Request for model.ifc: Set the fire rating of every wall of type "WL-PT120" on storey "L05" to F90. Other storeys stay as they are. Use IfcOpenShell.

First a look at what the model holds.

```python
import ifcopenshell
import ifcopenshell.util.element

model = ifcopenshell.open("model.ifc")
print(model.schema)
storey = next(s for s in model.by_type("IfcBuildingStorey") if s.Name == "L05")
walls = [e for e in ifcopenshell.util.element.get_decomposition(storey) if e.is_a("IfcWall")]
seen = {}
for e in walls:
    element_type = ifcopenshell.util.element.get_type(e)
    key = (element_type.Name if element_type != e and element_type else None, ifcopenshell.util.element.get_pset(e, "Pset_WallCommon", "FireRating"))
    seen[key] = seen.get(key, 0) + 1
for (name, value), count in sorted(seen.items(), key=str):
    print(count, "x", name, "|", value)
```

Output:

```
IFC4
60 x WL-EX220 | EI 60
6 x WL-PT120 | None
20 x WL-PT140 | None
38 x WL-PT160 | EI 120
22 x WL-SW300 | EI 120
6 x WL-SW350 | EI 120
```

```python
import ifcopenshell
import ifcopenshell.api.pset
import ifcopenshell.util.element

model = ifcopenshell.open("model.ifc")

storey = next(s for s in model.by_type("IfcBuildingStorey") if s.Name == "L05")
walls = [e for e in ifcopenshell.util.element.get_decomposition(storey) if e.is_a("IfcWall")]

count = 0
for e in walls:
    element_type = ifcopenshell.util.element.get_type(e)
    if element_type in (None, e) or element_type.Name != "WL-PT120":
        continue
    # add_pset returns the element's existing set when there is one.
    pset = ifcopenshell.api.pset.add_pset(model, product=e, name="Pset_WallCommon")
    ifcopenshell.api.pset.edit_pset(model, pset=pset, properties={"FireRating": "F90"})
    count += 1

print(count, "walls updated")

model.write("model_edited.ifc")
```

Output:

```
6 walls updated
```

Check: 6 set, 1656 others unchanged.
